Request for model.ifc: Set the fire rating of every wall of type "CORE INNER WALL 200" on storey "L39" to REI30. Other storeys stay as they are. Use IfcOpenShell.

First a look at what the model holds.

```python
import ifcopenshell
import ifcopenshell.util.element

model = ifcopenshell.open("model.ifc")
print(model.schema)
storey = next(s for s in model.by_type("IfcBuildingStorey") if s.Name == "L39")
walls = [e for e in ifcopenshell.util.element.get_decomposition(storey) if e.is_a("IfcWall")]
seen = {}
for e in walls:
    element_type = ifcopenshell.util.element.get_type(e)
    key = (element_type.Name if element_type != e and element_type else None, ifcopenshell.util.element.get_pset(e, "Pset_WallCommon", "FireRating"))
    seen[key] = seen.get(key, 0) + 1
for (name, value), count in sorted(seen.items(), key=str):
    print(count, "x", name, "|", value)
```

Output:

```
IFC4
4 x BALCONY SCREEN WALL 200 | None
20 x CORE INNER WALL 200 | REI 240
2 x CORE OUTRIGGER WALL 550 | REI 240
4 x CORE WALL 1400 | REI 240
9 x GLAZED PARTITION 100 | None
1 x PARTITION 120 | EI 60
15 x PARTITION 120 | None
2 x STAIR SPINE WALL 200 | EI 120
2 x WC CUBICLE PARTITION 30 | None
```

```python
import ifcopenshell
import ifcopenshell.api.pset
import ifcopenshell.util.element

model = ifcopenshell.open("model.ifc")

storey = next(s for s in model.by_type("IfcBuildingStorey") if s.Name == "L39")
walls = [e for e in ifcopenshell.util.element.get_decomposition(storey) if e.is_a("IfcWall")]

count = 0
for e in walls:
    element_type = ifcopenshell.util.element.get_type(e)
    if element_type in (None, e) or element_type.Name != "CORE INNER WALL 200":
        continue
    # add_pset returns the element's existing set when there is one.
    pset = ifcopenshell.api.pset.add_pset(model, product=e, name="Pset_WallCommon")
    ifcopenshell.api.pset.edit_pset(model, pset=pset, properties={"FireRating": "REI30"})
    count += 1

print(count, "walls updated")

model.write("model_updated.ifc")
```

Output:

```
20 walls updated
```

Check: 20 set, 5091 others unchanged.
